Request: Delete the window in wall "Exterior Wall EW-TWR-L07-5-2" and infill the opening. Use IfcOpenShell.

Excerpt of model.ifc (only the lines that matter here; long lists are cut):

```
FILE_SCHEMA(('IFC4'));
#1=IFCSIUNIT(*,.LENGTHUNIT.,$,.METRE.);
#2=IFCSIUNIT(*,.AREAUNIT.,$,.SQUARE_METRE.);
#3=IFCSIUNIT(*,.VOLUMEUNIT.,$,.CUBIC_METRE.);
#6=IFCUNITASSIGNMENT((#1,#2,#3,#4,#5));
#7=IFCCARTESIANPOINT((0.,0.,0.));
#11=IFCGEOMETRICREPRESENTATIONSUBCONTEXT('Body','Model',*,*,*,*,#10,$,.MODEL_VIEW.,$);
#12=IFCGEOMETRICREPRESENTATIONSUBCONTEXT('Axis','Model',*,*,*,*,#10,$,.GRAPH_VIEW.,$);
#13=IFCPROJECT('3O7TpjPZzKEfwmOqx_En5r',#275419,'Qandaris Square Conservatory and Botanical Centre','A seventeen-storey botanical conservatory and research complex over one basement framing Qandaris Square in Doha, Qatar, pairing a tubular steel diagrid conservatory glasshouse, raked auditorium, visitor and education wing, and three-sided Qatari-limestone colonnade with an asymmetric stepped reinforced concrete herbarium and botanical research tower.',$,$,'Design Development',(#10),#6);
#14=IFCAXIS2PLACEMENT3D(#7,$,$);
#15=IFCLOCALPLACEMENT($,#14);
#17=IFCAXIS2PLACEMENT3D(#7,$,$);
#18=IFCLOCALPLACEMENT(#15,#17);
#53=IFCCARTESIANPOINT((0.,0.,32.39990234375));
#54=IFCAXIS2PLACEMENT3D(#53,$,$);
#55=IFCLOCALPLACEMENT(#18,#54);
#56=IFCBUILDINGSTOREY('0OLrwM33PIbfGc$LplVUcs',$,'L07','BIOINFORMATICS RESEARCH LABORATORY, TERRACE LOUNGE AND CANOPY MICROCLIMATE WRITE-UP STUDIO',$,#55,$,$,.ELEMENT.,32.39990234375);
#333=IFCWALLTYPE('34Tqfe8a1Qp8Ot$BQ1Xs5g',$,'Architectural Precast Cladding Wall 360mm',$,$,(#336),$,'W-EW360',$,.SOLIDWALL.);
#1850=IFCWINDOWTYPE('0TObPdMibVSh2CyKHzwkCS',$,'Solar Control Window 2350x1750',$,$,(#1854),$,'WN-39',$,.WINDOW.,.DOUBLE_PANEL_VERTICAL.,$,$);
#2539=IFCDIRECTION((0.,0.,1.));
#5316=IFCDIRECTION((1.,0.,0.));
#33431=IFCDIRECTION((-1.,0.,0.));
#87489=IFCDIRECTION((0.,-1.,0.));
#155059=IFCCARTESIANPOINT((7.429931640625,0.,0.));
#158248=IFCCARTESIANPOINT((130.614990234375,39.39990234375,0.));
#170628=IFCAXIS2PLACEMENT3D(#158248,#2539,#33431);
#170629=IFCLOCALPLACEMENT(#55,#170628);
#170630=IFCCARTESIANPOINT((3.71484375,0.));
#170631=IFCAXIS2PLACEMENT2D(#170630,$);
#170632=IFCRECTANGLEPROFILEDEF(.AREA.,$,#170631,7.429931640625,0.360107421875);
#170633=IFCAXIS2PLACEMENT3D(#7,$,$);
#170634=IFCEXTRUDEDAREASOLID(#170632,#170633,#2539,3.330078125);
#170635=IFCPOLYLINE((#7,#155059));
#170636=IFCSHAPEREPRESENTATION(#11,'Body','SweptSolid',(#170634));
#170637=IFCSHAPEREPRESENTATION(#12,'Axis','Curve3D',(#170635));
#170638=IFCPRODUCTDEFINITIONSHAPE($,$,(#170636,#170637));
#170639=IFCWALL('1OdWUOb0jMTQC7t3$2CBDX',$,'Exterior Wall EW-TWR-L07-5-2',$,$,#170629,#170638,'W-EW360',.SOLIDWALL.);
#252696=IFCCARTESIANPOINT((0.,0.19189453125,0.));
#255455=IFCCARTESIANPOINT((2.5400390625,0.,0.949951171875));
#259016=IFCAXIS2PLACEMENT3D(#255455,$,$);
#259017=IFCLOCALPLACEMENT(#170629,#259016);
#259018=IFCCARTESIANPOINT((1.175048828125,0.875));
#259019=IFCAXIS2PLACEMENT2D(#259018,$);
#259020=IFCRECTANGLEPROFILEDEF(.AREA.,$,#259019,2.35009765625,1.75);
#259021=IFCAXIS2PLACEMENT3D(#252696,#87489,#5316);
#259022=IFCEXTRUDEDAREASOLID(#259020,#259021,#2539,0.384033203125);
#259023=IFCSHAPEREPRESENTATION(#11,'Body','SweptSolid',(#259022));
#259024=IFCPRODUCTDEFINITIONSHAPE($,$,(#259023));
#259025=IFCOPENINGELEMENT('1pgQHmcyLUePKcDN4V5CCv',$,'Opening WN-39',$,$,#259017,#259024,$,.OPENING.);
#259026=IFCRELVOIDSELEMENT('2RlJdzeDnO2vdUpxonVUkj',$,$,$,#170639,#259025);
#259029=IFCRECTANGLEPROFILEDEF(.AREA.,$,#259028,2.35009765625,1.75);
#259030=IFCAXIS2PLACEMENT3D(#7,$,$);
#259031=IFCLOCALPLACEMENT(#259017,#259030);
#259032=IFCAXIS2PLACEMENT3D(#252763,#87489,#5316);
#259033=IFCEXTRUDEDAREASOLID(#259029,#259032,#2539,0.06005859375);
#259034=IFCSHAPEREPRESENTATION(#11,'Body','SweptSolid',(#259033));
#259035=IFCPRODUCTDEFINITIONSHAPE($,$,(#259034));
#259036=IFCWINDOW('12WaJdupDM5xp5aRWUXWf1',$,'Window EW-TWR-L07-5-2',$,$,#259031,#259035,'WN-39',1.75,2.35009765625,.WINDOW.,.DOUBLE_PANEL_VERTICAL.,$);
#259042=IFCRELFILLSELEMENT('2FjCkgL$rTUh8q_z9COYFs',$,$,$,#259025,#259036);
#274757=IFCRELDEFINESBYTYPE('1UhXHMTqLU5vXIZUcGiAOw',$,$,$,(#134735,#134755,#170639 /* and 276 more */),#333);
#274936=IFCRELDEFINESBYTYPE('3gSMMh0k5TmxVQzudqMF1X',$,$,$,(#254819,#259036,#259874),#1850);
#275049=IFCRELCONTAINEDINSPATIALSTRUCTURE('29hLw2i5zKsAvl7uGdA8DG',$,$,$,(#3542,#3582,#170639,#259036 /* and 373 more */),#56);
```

```python
import ifcopenshell
import ifcopenshell.api.feature
import ifcopenshell.api.root
import ifcopenshell.geom
import ifcopenshell.util.shape

model = ifcopenshell.open("model.ifc")
settings = ifcopenshell.geom.settings()


def volume(element):
    """Net volume in cubic metres, openings subtracted."""
    shape = ifcopenshell.geom.create_shape(settings, element)
    return ifcopenshell.util.shape.get_volume(shape.geometry)


window = model.by_guid("12WaJdupDM5xp5aRWUXWf1")
opening = window.FillsVoids[0].RelatingOpeningElement
wall = opening.VoidsElements[0].RelatingBuildingElement
before = volume(wall)

ifcopenshell.api.root.remove_product(model, product=window)
ifcopenshell.api.feature.remove_feature(model, feature=opening)

after = volume(wall)

print(f"wall volume {before:.3f} -> {after:.3f} m3")

model.write("model_edited.ifc")
```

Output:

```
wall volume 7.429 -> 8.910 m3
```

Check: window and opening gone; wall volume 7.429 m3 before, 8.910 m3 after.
